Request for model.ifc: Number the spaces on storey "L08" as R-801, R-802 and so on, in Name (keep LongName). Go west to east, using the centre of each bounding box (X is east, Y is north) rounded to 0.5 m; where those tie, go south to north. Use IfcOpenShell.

First a look at what the model holds.

```python
import ifcopenshell
import ifcopenshell.util.element
import ifcopenshell.util.placement

model = ifcopenshell.open("model.ifc")
print(model.schema)
storey = next(s for s in model.by_type("IfcBuildingStorey") if s.Name == "L08")
spaces = [e for e in ifcopenshell.util.element.get_decomposition(storey) if e.is_a("IfcSpace")]
for e in sorted(spaces, key=lambda e: e.id()):
    origin = ifcopenshell.util.placement.get_local_placement(e.ObjectPlacement)[:3, 3]
    print(e.id(), e.Name, e.LongName, origin.round(2) + 0.0, sep=" | ")
```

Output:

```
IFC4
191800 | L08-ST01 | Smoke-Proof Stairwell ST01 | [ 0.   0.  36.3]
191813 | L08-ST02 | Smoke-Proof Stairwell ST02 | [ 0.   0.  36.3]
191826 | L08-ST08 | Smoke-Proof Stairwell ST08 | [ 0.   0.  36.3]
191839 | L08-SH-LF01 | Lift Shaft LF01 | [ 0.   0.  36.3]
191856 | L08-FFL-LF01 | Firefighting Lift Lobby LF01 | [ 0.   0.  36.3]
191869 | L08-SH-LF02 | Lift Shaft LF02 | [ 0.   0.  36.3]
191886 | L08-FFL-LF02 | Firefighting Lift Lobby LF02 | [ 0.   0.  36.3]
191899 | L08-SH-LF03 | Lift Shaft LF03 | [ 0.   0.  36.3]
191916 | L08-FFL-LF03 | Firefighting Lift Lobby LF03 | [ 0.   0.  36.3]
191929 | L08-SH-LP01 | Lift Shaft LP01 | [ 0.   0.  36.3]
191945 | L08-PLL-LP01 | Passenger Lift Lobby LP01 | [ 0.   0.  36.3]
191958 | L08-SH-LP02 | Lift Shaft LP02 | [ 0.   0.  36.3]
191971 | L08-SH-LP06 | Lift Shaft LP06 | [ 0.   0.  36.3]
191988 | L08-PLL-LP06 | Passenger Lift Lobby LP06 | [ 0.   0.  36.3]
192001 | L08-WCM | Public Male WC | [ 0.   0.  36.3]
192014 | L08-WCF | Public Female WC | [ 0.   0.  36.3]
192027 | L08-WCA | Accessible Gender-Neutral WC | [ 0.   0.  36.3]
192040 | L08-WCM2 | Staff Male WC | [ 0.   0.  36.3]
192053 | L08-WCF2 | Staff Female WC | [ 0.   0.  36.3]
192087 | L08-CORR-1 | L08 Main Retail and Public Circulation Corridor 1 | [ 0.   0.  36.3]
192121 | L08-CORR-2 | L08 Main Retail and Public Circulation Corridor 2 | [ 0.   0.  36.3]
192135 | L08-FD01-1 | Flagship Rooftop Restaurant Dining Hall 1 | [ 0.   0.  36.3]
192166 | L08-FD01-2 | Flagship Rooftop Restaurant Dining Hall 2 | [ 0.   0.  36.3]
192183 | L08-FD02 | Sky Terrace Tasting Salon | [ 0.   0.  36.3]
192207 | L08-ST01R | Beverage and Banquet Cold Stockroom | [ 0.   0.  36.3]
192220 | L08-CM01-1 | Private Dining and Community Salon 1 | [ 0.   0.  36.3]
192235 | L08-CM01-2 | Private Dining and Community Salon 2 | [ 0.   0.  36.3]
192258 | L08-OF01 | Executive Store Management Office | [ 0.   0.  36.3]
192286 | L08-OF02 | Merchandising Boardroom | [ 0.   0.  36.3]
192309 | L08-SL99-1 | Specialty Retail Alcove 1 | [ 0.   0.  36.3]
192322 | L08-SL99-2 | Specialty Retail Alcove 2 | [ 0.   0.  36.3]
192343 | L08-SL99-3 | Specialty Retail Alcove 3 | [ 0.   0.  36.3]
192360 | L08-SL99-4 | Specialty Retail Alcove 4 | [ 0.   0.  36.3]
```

```python
import ifcopenshell
import ifcopenshell.geom
import ifcopenshell.util.element
import ifcopenshell.util.shape

model = ifcopenshell.open("model.ifc")
settings = ifcopenshell.geom.settings()
settings.set("use-world-coords", True)


def centre(element):
    shape = ifcopenshell.geom.create_shape(settings, element)
    return ifcopenshell.util.shape.get_bbox_centroid(shape.geometry)


storey = next(s for s in model.by_type("IfcBuildingStorey") if s.Name == "L08")
spaces = [e for e in ifcopenshell.util.element.get_decomposition(storey) if e.is_a("IfcSpace")]

# Insertion points can sit at a corner or the storey origin, so sort by the geometry (in metres).
centres = {e: centre(e) for e in spaces}
spaces.sort(key=lambda e: (round(centres[e][0] / 0.5), centres[e][1]))

for i, e in enumerate(spaces, start=1):
    number = f"R-8{i:02d}"
    e.Name = number
    print(e.id(), number)

model.write("model_rev.ifc")
```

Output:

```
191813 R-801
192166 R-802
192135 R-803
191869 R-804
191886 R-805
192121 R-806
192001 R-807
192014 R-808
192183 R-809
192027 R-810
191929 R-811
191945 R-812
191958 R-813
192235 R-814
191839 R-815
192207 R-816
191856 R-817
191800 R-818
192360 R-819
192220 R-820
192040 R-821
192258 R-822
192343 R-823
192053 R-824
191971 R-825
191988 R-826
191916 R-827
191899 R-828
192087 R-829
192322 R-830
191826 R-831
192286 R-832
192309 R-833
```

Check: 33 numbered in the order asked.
